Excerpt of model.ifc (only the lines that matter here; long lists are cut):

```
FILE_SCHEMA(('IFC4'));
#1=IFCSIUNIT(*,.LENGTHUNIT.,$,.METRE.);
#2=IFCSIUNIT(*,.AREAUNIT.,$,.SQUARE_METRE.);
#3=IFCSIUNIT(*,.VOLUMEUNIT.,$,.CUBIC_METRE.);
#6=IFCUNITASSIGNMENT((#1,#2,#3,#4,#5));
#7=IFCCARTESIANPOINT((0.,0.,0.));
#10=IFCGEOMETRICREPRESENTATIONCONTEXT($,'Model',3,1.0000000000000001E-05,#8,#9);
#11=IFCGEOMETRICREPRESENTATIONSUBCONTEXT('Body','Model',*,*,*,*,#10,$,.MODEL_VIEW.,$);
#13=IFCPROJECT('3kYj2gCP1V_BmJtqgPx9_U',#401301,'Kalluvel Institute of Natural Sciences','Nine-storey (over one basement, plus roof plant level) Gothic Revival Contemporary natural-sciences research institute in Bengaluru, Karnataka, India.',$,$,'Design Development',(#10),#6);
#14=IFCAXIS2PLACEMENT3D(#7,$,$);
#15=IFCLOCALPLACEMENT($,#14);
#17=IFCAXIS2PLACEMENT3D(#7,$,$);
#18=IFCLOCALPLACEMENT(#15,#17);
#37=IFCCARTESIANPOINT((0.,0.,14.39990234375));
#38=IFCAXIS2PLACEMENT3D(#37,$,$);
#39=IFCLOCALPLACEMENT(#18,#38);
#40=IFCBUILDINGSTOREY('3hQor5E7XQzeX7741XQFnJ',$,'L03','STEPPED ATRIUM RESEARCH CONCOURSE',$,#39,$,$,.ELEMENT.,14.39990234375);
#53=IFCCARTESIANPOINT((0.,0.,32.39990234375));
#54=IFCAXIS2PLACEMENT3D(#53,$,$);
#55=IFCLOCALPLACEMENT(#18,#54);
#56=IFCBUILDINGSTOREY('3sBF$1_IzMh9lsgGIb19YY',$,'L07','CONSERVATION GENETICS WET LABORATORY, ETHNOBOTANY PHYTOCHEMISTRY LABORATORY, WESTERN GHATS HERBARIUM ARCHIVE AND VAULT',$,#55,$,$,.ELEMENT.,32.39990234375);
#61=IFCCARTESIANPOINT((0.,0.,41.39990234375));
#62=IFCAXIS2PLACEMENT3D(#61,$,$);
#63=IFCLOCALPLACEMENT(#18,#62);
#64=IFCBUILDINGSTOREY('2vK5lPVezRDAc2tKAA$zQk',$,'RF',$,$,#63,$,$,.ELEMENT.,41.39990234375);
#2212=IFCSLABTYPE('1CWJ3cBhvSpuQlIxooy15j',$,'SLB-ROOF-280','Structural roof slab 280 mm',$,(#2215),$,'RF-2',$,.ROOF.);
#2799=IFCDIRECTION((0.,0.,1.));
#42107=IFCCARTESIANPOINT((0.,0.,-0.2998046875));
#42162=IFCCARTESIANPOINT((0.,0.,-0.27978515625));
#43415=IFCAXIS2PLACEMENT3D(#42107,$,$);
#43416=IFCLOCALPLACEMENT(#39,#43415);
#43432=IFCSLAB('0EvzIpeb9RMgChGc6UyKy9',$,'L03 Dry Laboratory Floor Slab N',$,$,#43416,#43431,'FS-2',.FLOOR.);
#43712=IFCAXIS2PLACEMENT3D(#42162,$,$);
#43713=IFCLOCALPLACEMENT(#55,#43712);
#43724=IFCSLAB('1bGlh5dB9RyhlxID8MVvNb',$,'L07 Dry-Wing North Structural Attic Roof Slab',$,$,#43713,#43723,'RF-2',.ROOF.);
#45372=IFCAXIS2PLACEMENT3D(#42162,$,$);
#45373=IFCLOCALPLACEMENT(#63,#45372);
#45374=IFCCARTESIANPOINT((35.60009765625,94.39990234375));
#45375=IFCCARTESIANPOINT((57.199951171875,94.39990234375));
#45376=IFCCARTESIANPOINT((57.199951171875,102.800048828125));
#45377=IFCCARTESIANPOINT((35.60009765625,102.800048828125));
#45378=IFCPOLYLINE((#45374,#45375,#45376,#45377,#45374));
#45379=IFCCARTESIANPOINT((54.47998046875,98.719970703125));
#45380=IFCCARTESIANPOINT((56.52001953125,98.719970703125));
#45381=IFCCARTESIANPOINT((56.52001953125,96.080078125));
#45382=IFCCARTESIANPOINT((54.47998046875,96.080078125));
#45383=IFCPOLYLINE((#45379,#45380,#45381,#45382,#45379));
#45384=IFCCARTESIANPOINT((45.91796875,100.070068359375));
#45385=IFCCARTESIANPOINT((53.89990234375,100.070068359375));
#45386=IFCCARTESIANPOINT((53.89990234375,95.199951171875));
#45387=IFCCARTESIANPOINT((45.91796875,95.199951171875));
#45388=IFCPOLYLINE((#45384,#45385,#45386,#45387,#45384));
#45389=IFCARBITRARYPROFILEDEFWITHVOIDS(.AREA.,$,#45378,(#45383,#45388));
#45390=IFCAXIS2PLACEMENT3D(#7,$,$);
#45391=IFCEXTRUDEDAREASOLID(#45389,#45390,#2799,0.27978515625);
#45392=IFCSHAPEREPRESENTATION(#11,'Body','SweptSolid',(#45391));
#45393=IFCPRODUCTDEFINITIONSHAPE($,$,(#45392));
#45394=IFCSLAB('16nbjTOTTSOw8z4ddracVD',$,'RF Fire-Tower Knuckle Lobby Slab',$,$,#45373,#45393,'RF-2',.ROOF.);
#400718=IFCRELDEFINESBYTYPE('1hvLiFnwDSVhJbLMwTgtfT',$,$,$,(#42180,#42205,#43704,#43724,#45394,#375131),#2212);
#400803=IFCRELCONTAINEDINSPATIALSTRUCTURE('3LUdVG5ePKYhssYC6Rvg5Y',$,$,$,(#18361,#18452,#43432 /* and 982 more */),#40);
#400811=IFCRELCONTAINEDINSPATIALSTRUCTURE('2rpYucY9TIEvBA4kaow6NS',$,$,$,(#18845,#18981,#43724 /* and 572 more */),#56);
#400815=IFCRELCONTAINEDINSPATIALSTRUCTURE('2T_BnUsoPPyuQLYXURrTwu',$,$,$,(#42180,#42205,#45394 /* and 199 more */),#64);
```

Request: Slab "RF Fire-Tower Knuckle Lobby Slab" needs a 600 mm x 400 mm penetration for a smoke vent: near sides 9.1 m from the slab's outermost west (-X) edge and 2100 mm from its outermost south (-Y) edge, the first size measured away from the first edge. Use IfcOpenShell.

```python
import numpy as np
import ifcopenshell
import ifcopenshell.api.feature
import ifcopenshell.api.geometry
import ifcopenshell.api.root
import ifcopenshell.geom
import ifcopenshell.util.placement
import ifcopenshell.util.representation
import ifcopenshell.util.shape
import ifcopenshell.util.unit

model = ifcopenshell.open("model.ifc")
unit_scale = ifcopenshell.util.unit.calculate_unit_scale(model)
settings = ifcopenshell.geom.settings()


def volume(element):
    """Net volume in cubic metres, openings subtracted."""
    shape = ifcopenshell.geom.create_shape(settings, element)
    return ifcopenshell.util.shape.get_volume(shape.geometry)


slab = model.by_guid("16nbjTOTTSOw8z4ddracVD")
before = volume(slab)

# Extent in the slab's own axes, in metres. The edges named are its -X and -Y sides.
slab_shape = ifcopenshell.geom.create_shape(settings, slab)
vertices = ifcopenshell.util.shape.get_vertices(slab_shape.geometry)
x_min, y_min, bottom = vertices.min(axis=0)
top = vertices[:, 2].max()

opening = ifcopenshell.api.root.create_entity(model, ifc_class="IfcOpeningElement", name="Smoke vent opening", predefined_type="OPENING")
context = ifcopenshell.util.representation.get_context(model, "Model", "Body", "MODEL_VIEW")
width, depth = 0.6, 0.4
outline = [(0.0, 0.0), (width, 0.0), (width, depth), (0.0, depth), (0.0, 0.0)]
# Overshoot both faces by 50 mm so the cut is clean.
shape = ifcopenshell.api.geometry.add_slab_representation(
    model, context=context, depth=top - bottom + 0.1, polyline=outline
)
ifcopenshell.api.geometry.assign_representation(model, product=opening, representation=shape)

matrix = ifcopenshell.util.placement.get_local_placement(slab.ObjectPlacement)
matrix[:, 3] = matrix @ np.append(np.array([x_min + 9.1, y_min + 2.1, bottom - 0.05]) / unit_scale, 1.0)
ifcopenshell.api.geometry.edit_object_placement(model, product=opening, matrix=matrix, is_si=False)
ifcopenshell.api.feature.add_feature(model, feature=opening, element=slab)

after = volume(slab)

print(f"slab volume {before:.3f} -> {after:.3f} m3")

model.write("model_updated.ifc")
```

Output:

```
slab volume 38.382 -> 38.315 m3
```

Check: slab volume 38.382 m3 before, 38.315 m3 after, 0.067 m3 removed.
